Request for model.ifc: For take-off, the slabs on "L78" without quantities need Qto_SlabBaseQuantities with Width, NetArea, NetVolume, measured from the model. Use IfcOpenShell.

First a look at what the model holds.

```python
import ifcopenshell
import ifcopenshell.util.element
import ifcopenshell.util.unit

model = ifcopenshell.open("model.ifc")
print(model.schema)
for unit_type in ("LENGTHUNIT", "AREAUNIT", "VOLUMEUNIT"):
    print(unit_type, ifcopenshell.util.unit.calculate_unit_scale(model, unit_type))
storey = next(s for s in model.by_type("IfcBuildingStorey") if s.Name == "L78")
slabs = [e for e in ifcopenshell.util.element.get_decomposition(storey) if e.is_a("IfcSlab")]
for e in sorted(slabs, key=lambda e: e.id()):
    print(e.id(), e.is_a(), e.Name, list(ifcopenshell.util.element.get_psets(e, qtos_only=True)), sep=" | ")
```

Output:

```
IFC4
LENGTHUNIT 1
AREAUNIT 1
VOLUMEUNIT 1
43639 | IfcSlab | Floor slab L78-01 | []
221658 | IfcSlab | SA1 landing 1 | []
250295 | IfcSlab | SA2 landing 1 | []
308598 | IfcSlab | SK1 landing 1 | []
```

```python
import ifcopenshell
import ifcopenshell.api.pset
import ifcopenshell.geom
import ifcopenshell.util.element
import ifcopenshell.util.shape
import ifcopenshell.util.unit

model = ifcopenshell.open("model.ifc")
unit_scale = ifcopenshell.util.unit.calculate_unit_scale(model)
area_scale = ifcopenshell.util.unit.calculate_unit_scale(model, "AREAUNIT")
volume_scale = ifcopenshell.util.unit.calculate_unit_scale(model, "VOLUMEUNIT")
settings = ifcopenshell.geom.settings()

storey = next(s for s in model.by_type("IfcBuildingStorey") if s.Name == "L78")
slabs = [e for e in ifcopenshell.util.element.get_decomposition(storey) if e.is_a("IfcSlab")]

for e in sorted(slabs, key=lambda e: e.id()):
    if ifcopenshell.util.element.get_psets(e, qtos_only=True, should_inherit=False):
        continue
    # Geometry comes back in metres, in the element's own axes.
    shape = ifcopenshell.geom.create_shape(settings, e)
    values = {
        "Width": ifcopenshell.util.shape.get_z(shape.geometry) / unit_scale,
        "NetArea": ifcopenshell.util.shape.get_footprint_area(shape.geometry) / area_scale,
        "NetVolume": ifcopenshell.util.shape.get_volume(shape.geometry) / volume_scale,
    }
    qto = ifcopenshell.api.pset.add_qto(model, product=e, name="Qto_SlabBaseQuantities")
    ifcopenshell.api.pset.edit_qto(model, qto=qto, properties=values)
    print(e.id(), {k: round(v, 3) for k, v in values.items()})

model.write("model_edited.ifc")
```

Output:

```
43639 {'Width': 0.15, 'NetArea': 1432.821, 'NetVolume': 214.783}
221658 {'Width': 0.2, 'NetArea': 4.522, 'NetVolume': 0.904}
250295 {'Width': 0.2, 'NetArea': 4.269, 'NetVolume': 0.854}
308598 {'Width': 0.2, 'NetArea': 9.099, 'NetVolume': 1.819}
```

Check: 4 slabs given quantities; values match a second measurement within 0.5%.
